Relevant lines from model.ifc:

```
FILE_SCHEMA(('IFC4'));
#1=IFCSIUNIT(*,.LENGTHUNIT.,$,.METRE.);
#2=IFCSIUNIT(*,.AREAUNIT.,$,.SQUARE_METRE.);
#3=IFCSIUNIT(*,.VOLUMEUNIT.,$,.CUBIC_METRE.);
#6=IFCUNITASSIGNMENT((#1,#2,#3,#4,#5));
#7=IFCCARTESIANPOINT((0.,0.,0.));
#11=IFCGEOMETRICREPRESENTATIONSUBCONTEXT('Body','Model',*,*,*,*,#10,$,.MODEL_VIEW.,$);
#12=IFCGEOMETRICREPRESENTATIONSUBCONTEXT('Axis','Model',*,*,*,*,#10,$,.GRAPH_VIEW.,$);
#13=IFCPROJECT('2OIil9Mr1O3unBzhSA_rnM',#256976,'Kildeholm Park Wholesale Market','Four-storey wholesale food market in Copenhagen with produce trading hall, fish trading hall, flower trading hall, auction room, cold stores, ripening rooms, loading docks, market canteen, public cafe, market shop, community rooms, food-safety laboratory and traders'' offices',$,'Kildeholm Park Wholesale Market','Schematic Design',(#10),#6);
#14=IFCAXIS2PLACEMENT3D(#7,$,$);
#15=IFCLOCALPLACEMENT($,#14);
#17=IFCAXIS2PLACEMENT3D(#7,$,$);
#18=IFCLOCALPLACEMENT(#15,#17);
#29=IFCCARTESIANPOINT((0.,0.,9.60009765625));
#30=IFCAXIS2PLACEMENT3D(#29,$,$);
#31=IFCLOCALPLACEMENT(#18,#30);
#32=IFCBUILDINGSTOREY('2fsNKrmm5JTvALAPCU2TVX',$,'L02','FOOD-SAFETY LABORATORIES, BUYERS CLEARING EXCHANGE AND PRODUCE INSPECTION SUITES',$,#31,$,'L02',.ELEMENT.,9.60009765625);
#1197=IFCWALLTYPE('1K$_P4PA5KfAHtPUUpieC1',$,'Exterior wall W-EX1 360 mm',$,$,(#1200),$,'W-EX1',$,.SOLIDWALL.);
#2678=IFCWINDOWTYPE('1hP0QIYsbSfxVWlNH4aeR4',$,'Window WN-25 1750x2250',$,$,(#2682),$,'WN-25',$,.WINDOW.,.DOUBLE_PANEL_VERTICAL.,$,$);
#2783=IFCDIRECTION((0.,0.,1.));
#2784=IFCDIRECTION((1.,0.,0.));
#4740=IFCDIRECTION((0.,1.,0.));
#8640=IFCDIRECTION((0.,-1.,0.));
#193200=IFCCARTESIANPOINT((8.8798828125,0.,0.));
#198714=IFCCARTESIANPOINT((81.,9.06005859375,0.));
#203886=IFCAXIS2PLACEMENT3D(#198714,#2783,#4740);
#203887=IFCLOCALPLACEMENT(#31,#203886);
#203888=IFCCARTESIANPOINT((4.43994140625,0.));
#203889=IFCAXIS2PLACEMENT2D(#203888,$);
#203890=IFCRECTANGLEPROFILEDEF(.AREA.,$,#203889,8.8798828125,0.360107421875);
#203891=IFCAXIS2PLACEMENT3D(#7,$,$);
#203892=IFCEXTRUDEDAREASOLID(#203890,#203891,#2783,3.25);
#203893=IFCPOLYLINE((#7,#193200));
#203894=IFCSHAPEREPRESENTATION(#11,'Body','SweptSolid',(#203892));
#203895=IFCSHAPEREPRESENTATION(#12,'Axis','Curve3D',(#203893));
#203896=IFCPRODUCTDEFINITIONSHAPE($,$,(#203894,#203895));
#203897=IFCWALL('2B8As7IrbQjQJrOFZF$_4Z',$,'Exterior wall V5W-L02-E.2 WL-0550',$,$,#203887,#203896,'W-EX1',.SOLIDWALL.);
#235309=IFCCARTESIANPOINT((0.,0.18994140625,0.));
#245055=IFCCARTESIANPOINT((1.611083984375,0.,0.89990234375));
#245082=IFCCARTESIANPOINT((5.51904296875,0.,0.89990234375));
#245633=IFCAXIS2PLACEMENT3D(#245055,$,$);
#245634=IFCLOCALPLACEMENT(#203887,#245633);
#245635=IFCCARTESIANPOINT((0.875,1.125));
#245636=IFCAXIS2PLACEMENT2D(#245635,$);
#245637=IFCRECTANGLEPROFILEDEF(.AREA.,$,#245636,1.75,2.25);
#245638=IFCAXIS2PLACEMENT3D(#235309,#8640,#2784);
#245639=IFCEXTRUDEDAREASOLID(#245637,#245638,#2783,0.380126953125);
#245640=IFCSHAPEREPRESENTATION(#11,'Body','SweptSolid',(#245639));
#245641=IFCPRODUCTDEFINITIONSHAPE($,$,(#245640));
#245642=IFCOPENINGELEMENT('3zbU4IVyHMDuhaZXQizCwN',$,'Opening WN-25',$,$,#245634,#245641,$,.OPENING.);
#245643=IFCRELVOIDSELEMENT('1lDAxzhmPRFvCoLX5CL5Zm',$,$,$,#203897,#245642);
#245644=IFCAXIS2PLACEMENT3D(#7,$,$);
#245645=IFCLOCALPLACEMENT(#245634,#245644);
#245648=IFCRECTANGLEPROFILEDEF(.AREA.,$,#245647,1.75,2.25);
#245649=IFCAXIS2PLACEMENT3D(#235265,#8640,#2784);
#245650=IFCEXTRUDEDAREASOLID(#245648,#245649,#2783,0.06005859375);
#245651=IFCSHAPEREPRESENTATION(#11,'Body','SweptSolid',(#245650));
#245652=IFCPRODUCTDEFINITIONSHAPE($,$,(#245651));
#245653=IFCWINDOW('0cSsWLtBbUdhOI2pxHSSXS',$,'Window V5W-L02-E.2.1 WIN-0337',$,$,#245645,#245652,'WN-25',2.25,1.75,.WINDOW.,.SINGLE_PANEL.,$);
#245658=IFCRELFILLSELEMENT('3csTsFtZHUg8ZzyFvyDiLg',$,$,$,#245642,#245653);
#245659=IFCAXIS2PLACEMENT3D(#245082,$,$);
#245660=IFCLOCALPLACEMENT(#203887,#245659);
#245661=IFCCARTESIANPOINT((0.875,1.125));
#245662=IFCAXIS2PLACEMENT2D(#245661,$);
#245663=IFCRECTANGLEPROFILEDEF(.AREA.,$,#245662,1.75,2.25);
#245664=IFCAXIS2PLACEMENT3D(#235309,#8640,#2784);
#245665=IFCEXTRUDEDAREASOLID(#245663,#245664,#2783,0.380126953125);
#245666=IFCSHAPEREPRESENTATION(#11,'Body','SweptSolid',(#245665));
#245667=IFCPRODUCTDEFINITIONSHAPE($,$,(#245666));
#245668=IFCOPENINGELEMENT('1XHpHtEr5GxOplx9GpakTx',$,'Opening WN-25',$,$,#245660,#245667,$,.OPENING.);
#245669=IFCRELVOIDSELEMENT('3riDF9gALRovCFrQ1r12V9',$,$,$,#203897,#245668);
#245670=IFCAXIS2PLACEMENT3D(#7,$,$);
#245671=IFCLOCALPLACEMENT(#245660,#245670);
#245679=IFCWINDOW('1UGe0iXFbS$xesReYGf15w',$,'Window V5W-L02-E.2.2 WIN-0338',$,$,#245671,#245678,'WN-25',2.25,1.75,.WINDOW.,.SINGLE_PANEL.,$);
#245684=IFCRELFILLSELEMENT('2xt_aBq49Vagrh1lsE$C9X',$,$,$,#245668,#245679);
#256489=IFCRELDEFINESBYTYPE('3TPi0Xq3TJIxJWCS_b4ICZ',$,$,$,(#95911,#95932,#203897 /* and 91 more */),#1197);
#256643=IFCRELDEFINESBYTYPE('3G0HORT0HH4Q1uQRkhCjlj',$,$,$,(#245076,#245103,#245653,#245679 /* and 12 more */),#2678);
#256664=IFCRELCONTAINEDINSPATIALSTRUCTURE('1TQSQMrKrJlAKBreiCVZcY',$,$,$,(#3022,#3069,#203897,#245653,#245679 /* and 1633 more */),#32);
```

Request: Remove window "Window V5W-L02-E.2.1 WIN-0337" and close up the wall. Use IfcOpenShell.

```python
import ifcopenshell
import ifcopenshell.api.feature
import ifcopenshell.api.root
import ifcopenshell.geom
import ifcopenshell.util.shape

model = ifcopenshell.open("model.ifc")
settings = ifcopenshell.geom.settings()


def volume(element):
    """Net volume in cubic metres, openings subtracted."""
    shape = ifcopenshell.geom.create_shape(settings, element)
    return ifcopenshell.util.shape.get_volume(shape.geometry)


window = model.by_guid("0cSsWLtBbUdhOI2pxHSSXS")
opening = window.FillsVoids[0].RelatingOpeningElement
wall = opening.VoidsElements[0].RelatingBuildingElement
before = volume(wall)

ifcopenshell.api.root.remove_product(model, product=window)
ifcopenshell.api.feature.remove_feature(model, feature=opening)

after = volume(wall)

print(f"wall volume {before:.3f} -> {after:.3f} m3")

model.write("model_rev.ifc")
```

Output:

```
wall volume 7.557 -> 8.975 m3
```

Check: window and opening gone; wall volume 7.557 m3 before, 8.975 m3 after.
